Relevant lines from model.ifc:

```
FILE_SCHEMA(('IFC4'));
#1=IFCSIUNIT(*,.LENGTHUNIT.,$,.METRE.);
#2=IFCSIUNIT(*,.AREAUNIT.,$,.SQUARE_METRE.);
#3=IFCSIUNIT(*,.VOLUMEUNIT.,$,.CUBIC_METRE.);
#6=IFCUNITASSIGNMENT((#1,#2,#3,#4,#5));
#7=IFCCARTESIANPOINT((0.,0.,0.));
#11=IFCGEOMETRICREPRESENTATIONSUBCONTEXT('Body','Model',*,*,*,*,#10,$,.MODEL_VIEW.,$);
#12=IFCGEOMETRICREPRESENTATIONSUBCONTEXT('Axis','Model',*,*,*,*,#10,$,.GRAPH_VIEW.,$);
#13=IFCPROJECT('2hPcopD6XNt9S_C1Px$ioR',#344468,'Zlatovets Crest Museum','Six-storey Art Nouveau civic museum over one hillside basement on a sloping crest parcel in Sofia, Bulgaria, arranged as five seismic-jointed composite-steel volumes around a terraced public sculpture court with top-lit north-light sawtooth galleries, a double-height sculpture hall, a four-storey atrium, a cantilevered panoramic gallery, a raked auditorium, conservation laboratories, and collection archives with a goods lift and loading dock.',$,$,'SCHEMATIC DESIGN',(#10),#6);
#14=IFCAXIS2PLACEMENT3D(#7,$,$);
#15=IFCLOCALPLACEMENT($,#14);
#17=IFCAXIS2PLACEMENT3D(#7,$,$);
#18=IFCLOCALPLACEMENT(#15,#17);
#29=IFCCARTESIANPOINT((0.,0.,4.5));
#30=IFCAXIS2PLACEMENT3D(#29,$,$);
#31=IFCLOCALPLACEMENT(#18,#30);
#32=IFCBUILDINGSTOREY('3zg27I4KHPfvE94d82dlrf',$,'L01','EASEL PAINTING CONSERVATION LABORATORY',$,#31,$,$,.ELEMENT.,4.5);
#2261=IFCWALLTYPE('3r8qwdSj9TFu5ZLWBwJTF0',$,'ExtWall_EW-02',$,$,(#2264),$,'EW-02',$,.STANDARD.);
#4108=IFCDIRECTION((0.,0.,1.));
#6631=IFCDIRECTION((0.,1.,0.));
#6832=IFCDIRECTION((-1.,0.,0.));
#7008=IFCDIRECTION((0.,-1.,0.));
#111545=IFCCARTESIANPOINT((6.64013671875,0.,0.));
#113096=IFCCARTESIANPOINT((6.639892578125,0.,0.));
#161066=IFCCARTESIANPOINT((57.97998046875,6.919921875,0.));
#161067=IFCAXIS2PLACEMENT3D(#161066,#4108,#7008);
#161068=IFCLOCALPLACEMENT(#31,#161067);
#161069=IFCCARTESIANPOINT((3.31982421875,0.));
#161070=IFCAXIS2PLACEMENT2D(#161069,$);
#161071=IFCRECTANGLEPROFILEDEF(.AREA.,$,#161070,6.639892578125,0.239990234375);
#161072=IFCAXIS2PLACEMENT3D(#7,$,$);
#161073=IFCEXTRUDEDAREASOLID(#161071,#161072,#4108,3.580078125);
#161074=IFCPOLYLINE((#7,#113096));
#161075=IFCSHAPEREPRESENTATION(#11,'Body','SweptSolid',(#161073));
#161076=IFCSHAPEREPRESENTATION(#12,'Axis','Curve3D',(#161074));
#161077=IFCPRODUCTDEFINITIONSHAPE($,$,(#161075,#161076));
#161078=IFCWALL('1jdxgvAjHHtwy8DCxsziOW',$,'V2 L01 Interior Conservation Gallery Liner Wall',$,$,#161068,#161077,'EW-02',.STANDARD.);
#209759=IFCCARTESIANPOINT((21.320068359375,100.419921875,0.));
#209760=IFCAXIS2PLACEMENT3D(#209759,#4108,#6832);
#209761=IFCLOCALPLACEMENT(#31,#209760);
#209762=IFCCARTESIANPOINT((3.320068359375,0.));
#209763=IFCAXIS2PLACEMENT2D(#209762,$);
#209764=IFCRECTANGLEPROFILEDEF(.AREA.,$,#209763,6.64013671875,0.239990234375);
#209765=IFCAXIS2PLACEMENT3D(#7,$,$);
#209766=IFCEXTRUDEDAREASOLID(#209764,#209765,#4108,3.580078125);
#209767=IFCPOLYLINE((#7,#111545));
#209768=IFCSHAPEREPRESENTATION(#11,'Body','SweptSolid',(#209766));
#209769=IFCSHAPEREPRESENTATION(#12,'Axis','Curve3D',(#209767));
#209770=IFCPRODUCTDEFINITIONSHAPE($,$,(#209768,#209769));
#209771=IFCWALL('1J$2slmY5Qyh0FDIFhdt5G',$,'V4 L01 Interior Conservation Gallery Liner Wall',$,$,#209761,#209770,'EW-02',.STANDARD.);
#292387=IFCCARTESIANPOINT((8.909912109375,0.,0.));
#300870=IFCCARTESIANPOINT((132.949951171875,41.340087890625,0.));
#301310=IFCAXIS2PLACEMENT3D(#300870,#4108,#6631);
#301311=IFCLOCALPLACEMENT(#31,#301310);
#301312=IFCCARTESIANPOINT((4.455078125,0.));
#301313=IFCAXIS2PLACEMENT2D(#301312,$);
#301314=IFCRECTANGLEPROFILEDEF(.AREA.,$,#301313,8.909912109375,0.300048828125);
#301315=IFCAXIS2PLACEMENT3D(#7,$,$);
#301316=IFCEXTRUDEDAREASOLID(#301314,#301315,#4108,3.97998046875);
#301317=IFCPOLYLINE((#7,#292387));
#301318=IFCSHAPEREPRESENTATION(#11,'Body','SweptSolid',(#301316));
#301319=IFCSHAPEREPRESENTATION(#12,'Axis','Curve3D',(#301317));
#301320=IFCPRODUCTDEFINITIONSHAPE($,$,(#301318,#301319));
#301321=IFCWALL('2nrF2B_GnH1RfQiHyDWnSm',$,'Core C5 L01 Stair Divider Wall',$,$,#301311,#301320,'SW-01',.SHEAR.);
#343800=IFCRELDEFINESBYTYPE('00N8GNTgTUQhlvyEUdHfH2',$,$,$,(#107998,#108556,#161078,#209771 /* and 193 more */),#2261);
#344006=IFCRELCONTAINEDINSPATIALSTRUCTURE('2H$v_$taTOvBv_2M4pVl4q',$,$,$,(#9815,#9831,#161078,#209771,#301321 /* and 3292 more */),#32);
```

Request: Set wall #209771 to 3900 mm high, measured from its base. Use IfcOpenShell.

```python
import ifcopenshell
import ifcopenshell.geom
import ifcopenshell.util.representation
import ifcopenshell.util.shape
import ifcopenshell.util.unit

model = ifcopenshell.open("model.ifc")
unit_scale = ifcopenshell.util.unit.calculate_unit_scale(model)
settings = ifcopenshell.geom.settings()


def volume(element):
    """Net volume in cubic metres, openings subtracted."""
    shape = ifcopenshell.geom.create_shape(settings, element)
    return ifcopenshell.util.shape.get_volume(shape.geometry)


wall = model.by_guid("1J$2slmY5Qyh0FDIFhdt5G")
before = volume(wall)

body = ifcopenshell.util.representation.get_representation(wall, "Model", "Body")
solid = body.Items[0]
old_height = solid.Depth
solid.Depth = 3.9 / unit_scale
after = volume(wall)

print(f"height {old_height:g} -> {solid.Depth:g}, volume {before:.3f} -> {after:.3f} m3")

model.write("model_edited.ifc")
```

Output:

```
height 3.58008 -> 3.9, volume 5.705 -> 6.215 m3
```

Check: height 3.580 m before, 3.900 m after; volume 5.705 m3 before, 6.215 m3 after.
